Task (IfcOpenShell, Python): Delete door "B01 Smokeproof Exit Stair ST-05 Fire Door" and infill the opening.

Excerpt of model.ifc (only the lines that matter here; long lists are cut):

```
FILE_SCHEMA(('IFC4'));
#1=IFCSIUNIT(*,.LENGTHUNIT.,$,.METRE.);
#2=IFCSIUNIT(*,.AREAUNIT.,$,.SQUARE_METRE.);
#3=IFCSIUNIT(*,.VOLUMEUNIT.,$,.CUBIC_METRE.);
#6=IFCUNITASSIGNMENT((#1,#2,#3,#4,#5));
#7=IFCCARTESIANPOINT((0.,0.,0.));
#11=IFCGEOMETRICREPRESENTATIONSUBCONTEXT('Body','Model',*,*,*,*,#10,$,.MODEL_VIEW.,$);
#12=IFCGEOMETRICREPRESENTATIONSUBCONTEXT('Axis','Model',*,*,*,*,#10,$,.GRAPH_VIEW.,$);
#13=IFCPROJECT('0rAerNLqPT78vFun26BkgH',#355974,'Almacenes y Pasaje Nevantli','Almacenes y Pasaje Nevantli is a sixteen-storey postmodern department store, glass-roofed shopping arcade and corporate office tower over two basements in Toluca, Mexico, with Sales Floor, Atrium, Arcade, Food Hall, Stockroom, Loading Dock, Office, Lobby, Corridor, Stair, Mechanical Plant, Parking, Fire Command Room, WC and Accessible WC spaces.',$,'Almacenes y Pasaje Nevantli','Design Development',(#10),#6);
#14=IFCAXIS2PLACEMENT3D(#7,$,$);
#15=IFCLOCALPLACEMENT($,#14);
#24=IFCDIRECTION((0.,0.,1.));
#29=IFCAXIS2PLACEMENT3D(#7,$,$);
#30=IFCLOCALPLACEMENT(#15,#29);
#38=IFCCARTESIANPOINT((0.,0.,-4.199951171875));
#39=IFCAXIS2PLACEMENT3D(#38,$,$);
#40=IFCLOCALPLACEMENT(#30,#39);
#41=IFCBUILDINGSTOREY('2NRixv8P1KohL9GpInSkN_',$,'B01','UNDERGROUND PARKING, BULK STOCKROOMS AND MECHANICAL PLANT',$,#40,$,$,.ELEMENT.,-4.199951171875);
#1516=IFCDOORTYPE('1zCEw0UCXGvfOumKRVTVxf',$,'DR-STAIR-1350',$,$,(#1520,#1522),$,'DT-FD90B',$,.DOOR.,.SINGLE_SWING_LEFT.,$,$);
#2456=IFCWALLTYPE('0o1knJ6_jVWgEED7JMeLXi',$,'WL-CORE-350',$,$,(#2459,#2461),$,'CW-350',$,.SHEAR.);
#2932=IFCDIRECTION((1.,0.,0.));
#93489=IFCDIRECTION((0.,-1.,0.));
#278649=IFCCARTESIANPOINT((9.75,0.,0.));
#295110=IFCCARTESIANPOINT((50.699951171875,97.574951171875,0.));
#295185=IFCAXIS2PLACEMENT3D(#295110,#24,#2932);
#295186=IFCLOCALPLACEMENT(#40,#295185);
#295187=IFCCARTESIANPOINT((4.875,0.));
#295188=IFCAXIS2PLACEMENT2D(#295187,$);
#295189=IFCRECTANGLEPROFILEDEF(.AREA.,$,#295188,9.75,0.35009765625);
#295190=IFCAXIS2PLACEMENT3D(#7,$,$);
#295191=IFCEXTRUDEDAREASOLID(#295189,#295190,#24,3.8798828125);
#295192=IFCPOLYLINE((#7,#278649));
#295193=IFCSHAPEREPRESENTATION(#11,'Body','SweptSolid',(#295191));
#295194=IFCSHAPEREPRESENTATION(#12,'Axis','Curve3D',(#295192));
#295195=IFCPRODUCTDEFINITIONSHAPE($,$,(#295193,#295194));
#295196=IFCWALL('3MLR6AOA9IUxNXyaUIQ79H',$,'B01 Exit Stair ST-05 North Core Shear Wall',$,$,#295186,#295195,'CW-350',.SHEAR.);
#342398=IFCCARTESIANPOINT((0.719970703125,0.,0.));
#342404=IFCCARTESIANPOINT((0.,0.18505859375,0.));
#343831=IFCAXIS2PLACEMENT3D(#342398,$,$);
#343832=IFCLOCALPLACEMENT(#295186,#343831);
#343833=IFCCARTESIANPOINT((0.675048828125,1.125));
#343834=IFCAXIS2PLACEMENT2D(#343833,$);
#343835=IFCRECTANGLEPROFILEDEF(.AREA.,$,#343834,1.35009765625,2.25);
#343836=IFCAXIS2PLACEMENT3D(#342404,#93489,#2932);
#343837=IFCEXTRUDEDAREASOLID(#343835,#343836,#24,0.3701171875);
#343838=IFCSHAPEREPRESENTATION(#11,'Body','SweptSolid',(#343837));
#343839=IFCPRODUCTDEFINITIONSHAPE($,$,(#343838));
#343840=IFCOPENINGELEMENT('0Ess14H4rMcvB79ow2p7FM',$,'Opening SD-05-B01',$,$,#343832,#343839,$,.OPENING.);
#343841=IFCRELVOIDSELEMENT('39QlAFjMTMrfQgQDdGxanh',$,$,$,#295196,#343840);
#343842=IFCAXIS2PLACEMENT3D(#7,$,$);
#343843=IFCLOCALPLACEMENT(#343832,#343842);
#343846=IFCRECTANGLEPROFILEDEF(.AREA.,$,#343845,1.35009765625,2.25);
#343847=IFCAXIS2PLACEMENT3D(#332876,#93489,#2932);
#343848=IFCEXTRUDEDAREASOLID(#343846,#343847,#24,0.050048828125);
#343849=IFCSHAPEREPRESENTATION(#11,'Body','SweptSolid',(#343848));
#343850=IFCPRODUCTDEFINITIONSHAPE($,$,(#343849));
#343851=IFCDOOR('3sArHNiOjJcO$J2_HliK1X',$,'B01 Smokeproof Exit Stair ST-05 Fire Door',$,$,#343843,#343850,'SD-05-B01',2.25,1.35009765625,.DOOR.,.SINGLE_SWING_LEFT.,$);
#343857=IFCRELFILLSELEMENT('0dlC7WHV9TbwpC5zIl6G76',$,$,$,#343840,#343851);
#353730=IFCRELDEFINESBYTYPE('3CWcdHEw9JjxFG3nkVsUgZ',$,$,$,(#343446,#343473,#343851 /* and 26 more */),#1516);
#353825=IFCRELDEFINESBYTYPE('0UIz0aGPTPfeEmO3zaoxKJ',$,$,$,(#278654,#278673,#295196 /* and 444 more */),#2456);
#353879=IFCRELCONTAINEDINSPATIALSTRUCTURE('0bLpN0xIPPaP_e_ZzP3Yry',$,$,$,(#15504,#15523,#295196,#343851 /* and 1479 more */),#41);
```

```python
import ifcopenshell
import ifcopenshell.api.feature
import ifcopenshell.api.root
import ifcopenshell.geom
import ifcopenshell.util.shape

model = ifcopenshell.open("model.ifc")
settings = ifcopenshell.geom.settings()


def volume(element):
    """Net volume in cubic metres, openings subtracted."""
    shape = ifcopenshell.geom.create_shape(settings, element)
    return ifcopenshell.util.shape.get_volume(shape.geometry)


door = model.by_guid("3sArHNiOjJcO$J2_HliK1X")
opening = door.FillsVoids[0].RelatingOpeningElement
wall = opening.VoidsElements[0].RelatingBuildingElement
before = volume(wall)

ifcopenshell.api.root.remove_product(model, product=door)
ifcopenshell.api.feature.remove_feature(model, feature=opening)

after = volume(wall)

print(f"wall volume {before:.3f} -> {after:.3f} m3")

model.write("model_edited.ifc")
```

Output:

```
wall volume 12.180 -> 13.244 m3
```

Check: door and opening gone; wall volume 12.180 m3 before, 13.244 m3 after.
